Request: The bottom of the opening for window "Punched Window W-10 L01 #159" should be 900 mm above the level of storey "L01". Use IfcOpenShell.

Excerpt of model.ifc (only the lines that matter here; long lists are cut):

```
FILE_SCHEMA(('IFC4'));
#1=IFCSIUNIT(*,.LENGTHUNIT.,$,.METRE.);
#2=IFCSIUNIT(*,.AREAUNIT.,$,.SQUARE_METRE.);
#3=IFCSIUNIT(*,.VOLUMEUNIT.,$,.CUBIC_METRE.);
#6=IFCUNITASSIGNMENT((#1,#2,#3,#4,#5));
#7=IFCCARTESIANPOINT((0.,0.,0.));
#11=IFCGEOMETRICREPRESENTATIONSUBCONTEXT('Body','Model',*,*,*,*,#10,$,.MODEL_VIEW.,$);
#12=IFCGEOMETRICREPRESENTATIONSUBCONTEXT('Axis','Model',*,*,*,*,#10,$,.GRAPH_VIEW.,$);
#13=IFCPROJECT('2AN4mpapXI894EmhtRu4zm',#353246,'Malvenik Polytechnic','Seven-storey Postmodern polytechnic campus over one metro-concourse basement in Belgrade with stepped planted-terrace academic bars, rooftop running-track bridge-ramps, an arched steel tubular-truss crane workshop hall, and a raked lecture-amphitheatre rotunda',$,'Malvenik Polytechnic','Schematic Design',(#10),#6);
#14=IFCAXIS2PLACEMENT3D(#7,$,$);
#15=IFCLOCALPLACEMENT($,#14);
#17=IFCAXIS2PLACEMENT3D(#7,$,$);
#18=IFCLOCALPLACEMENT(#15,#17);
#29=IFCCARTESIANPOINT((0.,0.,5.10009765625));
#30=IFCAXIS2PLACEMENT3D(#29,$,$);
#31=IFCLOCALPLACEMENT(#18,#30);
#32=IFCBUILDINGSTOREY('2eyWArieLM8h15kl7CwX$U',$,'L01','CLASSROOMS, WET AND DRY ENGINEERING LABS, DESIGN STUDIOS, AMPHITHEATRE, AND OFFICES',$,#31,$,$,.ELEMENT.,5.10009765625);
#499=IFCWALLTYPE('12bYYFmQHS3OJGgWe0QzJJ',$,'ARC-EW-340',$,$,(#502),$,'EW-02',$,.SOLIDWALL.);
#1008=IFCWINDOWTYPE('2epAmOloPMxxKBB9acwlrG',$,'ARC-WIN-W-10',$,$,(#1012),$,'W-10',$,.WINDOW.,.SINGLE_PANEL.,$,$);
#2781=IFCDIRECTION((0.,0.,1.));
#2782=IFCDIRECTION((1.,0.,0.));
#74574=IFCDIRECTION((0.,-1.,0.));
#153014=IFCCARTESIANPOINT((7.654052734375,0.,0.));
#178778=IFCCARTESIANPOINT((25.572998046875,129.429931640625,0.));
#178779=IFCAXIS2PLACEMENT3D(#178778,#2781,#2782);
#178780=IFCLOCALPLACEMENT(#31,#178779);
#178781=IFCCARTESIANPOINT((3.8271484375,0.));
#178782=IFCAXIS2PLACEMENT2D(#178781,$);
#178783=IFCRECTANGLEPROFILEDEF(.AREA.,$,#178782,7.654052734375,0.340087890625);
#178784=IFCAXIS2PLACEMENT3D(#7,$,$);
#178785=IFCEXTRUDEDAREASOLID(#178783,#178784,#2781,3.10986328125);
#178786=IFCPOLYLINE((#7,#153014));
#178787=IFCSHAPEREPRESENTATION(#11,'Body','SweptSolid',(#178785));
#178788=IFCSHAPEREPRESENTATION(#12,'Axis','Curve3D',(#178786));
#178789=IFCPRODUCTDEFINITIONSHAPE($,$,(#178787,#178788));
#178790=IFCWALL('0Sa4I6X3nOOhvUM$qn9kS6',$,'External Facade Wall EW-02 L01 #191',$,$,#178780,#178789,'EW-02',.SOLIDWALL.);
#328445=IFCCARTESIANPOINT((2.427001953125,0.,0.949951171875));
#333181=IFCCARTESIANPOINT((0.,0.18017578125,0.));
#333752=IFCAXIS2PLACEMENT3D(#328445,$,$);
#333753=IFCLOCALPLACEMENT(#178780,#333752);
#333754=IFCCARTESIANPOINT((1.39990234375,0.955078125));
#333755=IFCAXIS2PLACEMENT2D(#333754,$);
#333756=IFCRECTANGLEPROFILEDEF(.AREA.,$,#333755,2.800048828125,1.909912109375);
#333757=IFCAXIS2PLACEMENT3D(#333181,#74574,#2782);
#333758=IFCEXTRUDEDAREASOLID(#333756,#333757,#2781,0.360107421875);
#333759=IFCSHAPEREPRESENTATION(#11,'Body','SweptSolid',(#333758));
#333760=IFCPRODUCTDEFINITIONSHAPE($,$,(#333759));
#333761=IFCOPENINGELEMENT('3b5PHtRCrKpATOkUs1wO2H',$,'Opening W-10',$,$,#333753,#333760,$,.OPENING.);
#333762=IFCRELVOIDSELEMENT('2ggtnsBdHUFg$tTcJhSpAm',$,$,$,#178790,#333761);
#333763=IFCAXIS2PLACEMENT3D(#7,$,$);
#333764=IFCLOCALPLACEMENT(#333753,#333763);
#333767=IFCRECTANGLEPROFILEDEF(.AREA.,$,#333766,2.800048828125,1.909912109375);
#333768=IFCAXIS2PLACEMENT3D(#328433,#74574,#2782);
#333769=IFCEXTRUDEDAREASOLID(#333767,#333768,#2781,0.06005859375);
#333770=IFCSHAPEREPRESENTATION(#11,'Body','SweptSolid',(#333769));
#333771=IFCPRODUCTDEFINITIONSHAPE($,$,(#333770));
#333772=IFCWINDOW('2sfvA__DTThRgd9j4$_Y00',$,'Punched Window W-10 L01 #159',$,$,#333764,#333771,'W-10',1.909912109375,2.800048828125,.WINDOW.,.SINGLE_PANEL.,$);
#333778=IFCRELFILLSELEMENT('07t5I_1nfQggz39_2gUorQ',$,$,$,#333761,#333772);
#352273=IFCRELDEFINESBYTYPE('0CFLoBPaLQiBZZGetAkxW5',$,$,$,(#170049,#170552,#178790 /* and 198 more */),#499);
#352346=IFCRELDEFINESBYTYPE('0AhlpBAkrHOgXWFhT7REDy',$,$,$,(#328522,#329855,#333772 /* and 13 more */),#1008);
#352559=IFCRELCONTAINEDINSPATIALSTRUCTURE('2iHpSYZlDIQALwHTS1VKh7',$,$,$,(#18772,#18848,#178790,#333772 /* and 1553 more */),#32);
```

```python
import numpy as np
import ifcopenshell
import ifcopenshell.api.geometry
import ifcopenshell.geom
import ifcopenshell.util.element
import ifcopenshell.util.placement
import ifcopenshell.util.shape
import ifcopenshell.util.unit

model = ifcopenshell.open("model.ifc")
unit_scale = ifcopenshell.util.unit.calculate_unit_scale(model)

window = model.by_id(333772)
opening = window.FillsVoids[0].RelatingOpeningElement
storey = ifcopenshell.util.element.get_container(window, ifc_class="IfcBuildingStorey")
level = ifcopenshell.util.placement.get_local_placement(storey.ObjectPlacement)[2, 3]

# The opening's origin need not be at the sill, so measure its lowest point.
shape = ifcopenshell.geom.create_shape(ifcopenshell.geom.settings(), opening)
bottom = ifcopenshell.util.shape.get_shape_bottom_elevation(shape, shape.geometry) / unit_scale
dz = level + 0.9 / unit_scale - bottom

shift = np.array([0.0, 0.0, dz])
# The window is placed relative to its opening, so it follows when the opening moves.
matrix = ifcopenshell.util.placement.get_local_placement(opening.ObjectPlacement)
matrix[:3, 3] += shift
ifcopenshell.api.geometry.edit_object_placement(
    model, product=opening, matrix=matrix, is_si=False, should_transform_children=True
)

print(f"moved by {dz * unit_scale:+.3f} m")

model.write("model_v2.ifc")
```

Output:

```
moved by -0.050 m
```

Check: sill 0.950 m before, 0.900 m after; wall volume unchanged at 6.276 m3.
